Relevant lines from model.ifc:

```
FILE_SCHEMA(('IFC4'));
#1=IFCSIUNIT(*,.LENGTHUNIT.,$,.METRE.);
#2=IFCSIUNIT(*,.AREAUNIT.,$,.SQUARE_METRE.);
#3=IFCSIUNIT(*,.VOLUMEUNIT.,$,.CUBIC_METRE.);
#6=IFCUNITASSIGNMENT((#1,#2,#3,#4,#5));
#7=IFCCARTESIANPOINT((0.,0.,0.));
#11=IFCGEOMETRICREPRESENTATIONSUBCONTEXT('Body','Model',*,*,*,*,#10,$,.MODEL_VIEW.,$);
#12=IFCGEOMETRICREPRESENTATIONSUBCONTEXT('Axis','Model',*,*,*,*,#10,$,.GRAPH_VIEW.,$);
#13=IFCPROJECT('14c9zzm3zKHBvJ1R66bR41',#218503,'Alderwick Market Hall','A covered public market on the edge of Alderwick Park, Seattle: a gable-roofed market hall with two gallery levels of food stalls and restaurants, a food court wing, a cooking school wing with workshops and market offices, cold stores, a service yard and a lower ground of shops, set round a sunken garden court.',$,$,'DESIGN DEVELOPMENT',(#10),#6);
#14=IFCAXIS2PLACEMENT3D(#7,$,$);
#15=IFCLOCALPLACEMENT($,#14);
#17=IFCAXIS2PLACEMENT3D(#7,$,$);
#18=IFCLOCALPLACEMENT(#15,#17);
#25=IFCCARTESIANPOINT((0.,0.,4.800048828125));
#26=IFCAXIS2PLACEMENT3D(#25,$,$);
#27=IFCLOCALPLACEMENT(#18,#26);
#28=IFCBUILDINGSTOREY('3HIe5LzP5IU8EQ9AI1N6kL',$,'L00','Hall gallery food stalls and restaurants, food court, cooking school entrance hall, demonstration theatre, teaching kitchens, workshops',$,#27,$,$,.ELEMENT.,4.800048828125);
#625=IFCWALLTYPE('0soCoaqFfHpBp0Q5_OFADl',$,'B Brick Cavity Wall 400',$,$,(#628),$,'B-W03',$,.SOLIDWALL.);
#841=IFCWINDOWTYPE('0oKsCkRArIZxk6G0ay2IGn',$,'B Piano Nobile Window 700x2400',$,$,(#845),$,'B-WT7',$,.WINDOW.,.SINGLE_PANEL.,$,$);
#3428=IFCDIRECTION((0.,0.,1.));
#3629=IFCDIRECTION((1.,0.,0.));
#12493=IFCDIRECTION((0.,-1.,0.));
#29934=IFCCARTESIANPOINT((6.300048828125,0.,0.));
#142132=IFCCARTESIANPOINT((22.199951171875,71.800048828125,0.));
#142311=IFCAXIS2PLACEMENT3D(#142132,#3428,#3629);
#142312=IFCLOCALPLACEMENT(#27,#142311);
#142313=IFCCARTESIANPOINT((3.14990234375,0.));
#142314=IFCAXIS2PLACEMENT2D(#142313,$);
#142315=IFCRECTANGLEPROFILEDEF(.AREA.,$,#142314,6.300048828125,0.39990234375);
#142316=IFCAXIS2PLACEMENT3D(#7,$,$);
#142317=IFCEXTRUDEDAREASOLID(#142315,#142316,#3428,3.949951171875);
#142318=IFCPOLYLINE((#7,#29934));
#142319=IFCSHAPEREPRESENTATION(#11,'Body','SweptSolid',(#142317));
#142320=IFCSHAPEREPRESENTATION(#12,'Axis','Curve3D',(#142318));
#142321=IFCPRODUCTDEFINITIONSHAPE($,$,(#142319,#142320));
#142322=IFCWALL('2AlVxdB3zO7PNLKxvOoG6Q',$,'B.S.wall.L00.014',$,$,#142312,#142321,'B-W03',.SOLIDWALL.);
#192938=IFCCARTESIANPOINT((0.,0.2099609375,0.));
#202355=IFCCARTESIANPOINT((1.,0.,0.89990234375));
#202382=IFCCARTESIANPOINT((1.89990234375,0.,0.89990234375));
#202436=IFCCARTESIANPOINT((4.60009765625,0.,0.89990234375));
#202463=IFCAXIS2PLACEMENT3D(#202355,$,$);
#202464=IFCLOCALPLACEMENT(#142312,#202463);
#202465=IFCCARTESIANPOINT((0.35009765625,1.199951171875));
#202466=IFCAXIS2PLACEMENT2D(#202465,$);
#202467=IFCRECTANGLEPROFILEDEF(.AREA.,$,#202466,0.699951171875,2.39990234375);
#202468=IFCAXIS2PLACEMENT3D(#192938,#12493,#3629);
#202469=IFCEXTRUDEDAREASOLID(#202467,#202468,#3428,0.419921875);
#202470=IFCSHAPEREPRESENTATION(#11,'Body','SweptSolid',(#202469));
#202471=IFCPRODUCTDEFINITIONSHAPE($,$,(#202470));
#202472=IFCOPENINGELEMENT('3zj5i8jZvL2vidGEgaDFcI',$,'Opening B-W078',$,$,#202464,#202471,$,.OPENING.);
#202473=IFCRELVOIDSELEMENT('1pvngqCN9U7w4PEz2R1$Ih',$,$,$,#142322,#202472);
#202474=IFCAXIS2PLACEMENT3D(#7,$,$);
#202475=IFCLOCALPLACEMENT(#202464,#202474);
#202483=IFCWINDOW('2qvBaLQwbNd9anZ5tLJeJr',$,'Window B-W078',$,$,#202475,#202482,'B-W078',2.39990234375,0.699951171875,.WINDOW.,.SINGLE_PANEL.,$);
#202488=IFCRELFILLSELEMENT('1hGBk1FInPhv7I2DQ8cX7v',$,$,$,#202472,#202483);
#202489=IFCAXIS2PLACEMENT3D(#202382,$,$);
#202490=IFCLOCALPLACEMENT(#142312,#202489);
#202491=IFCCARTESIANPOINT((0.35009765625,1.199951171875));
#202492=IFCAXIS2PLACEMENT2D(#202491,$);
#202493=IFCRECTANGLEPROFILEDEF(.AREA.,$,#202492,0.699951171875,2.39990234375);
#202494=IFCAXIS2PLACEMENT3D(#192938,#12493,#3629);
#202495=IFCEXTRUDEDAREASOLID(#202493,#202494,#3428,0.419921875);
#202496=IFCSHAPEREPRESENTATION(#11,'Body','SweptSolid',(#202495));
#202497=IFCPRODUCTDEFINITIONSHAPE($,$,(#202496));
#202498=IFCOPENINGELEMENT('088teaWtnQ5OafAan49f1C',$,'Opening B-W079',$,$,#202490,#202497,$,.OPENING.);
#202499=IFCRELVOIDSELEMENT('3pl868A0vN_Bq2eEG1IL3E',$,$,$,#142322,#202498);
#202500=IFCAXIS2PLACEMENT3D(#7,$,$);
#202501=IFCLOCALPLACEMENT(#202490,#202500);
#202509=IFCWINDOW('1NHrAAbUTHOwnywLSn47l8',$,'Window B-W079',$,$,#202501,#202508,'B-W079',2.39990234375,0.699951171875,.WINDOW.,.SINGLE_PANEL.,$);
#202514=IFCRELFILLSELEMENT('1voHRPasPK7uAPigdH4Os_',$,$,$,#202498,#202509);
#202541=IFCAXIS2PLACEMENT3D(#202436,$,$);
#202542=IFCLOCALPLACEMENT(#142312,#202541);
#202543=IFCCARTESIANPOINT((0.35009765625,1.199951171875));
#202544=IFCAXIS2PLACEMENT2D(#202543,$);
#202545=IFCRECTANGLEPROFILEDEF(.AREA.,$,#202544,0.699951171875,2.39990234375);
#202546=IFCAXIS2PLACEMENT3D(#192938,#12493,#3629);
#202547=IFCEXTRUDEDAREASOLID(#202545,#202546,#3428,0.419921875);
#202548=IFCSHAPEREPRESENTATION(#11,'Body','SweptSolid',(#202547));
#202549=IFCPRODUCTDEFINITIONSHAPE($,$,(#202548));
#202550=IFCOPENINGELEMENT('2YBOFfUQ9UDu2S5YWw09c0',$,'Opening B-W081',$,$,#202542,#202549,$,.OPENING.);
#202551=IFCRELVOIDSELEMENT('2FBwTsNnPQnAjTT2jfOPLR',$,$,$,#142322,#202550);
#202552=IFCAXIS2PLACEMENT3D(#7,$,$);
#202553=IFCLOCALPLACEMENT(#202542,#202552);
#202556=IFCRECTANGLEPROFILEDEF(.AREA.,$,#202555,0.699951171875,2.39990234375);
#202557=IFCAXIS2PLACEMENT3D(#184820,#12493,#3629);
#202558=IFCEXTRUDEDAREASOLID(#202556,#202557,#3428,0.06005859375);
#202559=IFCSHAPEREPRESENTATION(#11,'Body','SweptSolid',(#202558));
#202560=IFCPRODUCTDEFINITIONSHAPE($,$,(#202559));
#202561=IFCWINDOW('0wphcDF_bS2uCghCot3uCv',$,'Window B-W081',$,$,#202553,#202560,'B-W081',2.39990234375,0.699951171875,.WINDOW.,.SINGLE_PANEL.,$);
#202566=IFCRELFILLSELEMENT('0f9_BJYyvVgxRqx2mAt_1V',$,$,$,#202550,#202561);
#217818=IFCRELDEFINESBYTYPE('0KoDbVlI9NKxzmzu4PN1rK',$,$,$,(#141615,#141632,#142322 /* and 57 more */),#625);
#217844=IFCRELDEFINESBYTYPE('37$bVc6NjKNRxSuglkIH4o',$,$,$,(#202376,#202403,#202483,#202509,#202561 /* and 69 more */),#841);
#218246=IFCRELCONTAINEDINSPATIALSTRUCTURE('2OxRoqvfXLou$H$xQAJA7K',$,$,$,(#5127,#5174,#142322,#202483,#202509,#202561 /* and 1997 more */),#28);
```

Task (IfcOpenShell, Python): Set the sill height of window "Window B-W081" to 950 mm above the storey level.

```python
import numpy as np
import ifcopenshell
import ifcopenshell.api.geometry
import ifcopenshell.geom
import ifcopenshell.util.element
import ifcopenshell.util.placement
import ifcopenshell.util.shape
import ifcopenshell.util.unit

model = ifcopenshell.open("model.ifc")
unit_scale = ifcopenshell.util.unit.calculate_unit_scale(model)

window = model.by_id(202561)
opening = window.FillsVoids[0].RelatingOpeningElement
storey = ifcopenshell.util.element.get_container(window, ifc_class="IfcBuildingStorey")
level = ifcopenshell.util.placement.get_local_placement(storey.ObjectPlacement)[2, 3]

# The opening's origin need not be at the sill, so measure its lowest point.
shape = ifcopenshell.geom.create_shape(ifcopenshell.geom.settings(), opening)
bottom = ifcopenshell.util.shape.get_shape_bottom_elevation(shape, shape.geometry) / unit_scale
dz = level + 0.95 / unit_scale - bottom

shift = np.array([0.0, 0.0, dz])
# The window is placed relative to its opening, so it follows when the opening moves.
matrix = ifcopenshell.util.placement.get_local_placement(opening.ObjectPlacement)
matrix[:3, 3] += shift
ifcopenshell.api.geometry.edit_object_placement(
    model, product=opening, matrix=matrix, is_si=False, should_transform_children=True
)

print(f"moved by {dz * unit_scale:+.3f} m")

model.write("model_rev.ifc")
```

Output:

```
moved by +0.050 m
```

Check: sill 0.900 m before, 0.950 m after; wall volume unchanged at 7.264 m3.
